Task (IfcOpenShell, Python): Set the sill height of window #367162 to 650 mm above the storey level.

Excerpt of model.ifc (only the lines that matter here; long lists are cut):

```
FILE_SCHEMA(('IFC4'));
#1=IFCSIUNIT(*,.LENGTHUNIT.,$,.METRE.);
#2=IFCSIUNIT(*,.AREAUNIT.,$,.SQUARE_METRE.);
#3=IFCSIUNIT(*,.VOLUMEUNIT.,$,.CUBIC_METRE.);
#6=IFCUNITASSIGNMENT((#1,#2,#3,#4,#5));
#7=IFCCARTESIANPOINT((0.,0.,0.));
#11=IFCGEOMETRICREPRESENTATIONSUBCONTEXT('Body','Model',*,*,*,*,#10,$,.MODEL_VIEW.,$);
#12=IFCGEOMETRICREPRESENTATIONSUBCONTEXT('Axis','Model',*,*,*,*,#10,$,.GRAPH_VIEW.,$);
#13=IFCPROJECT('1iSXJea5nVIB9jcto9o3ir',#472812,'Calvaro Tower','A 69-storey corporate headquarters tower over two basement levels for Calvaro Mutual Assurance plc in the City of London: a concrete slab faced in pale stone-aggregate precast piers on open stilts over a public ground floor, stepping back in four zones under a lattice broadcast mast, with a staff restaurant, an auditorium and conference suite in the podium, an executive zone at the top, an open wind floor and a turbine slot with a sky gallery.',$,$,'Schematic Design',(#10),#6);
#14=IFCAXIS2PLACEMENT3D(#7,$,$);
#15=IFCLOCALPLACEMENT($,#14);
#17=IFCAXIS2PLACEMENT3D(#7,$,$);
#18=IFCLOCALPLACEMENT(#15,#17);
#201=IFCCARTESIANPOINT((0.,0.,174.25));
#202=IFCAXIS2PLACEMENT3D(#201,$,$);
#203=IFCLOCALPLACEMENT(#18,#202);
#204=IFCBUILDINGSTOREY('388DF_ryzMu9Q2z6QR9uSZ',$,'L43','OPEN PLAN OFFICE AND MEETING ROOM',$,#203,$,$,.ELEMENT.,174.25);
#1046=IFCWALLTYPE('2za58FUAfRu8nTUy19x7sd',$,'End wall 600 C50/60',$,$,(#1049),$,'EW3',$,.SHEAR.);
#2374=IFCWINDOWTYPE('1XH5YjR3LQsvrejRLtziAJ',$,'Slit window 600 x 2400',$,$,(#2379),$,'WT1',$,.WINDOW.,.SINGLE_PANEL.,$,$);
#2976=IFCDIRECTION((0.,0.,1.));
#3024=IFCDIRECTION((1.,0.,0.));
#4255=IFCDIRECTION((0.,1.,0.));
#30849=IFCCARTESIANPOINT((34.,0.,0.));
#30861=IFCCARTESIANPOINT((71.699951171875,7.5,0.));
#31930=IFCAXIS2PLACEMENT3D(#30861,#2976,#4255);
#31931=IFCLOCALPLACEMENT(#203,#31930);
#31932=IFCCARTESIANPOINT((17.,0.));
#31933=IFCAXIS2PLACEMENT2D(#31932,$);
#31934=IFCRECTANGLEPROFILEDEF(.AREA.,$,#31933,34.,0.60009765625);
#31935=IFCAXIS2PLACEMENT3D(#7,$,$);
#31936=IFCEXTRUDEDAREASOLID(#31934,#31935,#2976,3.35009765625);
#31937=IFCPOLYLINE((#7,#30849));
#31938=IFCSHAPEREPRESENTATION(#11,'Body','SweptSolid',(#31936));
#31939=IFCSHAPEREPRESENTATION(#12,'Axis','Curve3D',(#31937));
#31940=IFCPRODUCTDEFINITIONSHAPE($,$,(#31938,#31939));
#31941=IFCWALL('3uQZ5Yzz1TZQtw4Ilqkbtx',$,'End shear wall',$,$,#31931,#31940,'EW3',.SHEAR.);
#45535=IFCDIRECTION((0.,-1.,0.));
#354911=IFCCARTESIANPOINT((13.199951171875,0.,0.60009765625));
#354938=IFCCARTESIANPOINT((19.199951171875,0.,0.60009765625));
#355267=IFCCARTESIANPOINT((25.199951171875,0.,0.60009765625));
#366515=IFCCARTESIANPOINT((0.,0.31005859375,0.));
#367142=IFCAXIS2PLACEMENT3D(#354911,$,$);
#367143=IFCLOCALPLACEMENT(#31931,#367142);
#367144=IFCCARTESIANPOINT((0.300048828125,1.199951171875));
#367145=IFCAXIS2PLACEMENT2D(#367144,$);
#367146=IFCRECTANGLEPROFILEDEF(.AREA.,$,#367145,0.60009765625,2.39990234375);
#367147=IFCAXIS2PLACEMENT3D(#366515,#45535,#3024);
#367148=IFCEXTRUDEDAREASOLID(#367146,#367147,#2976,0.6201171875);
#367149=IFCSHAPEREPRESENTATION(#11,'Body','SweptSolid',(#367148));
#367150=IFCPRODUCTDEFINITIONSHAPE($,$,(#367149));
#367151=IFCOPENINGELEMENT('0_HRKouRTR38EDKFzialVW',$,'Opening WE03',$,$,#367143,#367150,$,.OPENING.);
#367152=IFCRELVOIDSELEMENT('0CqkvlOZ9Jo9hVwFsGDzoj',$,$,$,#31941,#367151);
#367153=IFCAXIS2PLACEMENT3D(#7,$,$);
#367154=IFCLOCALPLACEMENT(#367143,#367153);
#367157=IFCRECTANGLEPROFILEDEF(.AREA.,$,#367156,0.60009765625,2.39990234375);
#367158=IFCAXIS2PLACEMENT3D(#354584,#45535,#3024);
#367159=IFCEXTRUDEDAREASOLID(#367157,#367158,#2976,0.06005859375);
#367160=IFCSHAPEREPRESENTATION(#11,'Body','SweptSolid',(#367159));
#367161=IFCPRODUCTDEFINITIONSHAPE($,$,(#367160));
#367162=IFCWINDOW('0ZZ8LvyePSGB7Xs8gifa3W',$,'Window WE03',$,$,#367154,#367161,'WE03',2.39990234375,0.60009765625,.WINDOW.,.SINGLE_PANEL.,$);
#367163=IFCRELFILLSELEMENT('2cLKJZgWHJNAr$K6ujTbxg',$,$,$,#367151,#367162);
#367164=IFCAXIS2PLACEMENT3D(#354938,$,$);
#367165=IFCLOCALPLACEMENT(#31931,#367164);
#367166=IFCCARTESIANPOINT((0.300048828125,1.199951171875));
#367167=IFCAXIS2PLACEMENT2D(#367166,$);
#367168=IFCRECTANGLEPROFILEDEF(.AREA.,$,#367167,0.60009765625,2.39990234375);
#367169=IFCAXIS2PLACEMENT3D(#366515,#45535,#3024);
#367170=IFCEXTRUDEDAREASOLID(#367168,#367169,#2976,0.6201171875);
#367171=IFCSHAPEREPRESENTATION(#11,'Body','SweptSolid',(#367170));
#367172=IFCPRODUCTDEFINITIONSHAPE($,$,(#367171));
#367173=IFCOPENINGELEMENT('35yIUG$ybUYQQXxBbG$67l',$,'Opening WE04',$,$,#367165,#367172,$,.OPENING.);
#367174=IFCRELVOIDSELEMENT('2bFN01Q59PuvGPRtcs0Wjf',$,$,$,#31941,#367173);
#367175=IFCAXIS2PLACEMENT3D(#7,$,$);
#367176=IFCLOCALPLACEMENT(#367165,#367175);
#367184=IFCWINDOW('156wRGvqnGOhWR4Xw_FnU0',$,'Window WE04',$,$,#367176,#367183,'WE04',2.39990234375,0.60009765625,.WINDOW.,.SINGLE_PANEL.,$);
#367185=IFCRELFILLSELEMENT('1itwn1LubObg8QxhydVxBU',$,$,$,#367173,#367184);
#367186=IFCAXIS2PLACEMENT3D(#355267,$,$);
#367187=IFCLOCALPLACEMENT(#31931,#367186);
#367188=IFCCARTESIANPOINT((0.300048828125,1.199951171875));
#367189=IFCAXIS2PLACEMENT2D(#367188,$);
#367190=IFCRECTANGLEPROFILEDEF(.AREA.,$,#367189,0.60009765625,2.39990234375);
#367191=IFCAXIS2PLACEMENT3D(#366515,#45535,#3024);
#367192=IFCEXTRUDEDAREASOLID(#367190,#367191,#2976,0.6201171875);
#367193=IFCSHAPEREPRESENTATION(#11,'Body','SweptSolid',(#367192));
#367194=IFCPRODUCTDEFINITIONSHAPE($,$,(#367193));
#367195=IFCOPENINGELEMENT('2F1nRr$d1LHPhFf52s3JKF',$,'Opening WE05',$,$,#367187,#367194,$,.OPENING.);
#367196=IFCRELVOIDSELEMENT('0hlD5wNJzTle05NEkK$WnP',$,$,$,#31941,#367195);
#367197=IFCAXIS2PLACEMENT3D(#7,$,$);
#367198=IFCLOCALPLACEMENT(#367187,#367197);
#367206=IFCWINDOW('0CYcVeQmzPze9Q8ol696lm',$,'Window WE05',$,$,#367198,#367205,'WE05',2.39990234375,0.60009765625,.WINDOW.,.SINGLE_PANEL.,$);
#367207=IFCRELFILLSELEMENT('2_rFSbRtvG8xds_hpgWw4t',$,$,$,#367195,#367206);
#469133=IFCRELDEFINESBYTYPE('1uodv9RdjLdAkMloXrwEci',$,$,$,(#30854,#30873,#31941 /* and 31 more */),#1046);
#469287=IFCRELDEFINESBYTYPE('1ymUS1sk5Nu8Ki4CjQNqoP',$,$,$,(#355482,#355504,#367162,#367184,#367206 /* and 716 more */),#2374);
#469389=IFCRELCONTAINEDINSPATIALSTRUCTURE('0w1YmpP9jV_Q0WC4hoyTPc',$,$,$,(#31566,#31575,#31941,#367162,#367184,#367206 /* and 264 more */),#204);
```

```python
import numpy as np
import ifcopenshell
import ifcopenshell.api.geometry
import ifcopenshell.geom
import ifcopenshell.util.element
import ifcopenshell.util.placement
import ifcopenshell.util.shape
import ifcopenshell.util.unit

model = ifcopenshell.open("model.ifc")
unit_scale = ifcopenshell.util.unit.calculate_unit_scale(model)

window = model.by_id(367162)
opening = window.FillsVoids[0].RelatingOpeningElement
storey = ifcopenshell.util.element.get_container(window, ifc_class="IfcBuildingStorey")
level = ifcopenshell.util.placement.get_local_placement(storey.ObjectPlacement)[2, 3]

# The opening's origin need not be at the sill, so measure its lowest point.
shape = ifcopenshell.geom.create_shape(ifcopenshell.geom.settings(), opening)
bottom = ifcopenshell.util.shape.get_shape_bottom_elevation(shape, shape.geometry) / unit_scale
dz = level + 0.65 - bottom

shift = np.array([0.0, 0.0, dz])
# The window is placed relative to its opening, so it follows when the opening moves.
matrix = ifcopenshell.util.placement.get_local_placement(opening.ObjectPlacement)
matrix[:3, 3] += shift
ifcopenshell.api.geometry.edit_object_placement(
    model, product=opening, matrix=matrix, is_si=False, should_transform_children=True
)

print(f"moved by {dz * unit_scale:+.3f} m")

model.write("model_rev.ifc")
```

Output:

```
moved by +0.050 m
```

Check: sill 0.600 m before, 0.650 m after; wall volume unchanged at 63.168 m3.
